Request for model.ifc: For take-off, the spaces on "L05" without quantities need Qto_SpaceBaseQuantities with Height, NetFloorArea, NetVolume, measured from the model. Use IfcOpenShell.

First a look at what the model holds.

```python
import ifcopenshell
import ifcopenshell.util.element
import ifcopenshell.util.unit

model = ifcopenshell.open("model.ifc")
print(model.schema)
for unit_type in ("LENGTHUNIT", "AREAUNIT", "VOLUMEUNIT"):
    print(unit_type, ifcopenshell.util.unit.calculate_unit_scale(model, unit_type))
storey = next(s for s in model.by_type("IfcBuildingStorey") if s.Name == "L05")
spaces = [e for e in ifcopenshell.util.element.get_decomposition(storey) if e.is_a("IfcSpace")]
for e in sorted(spaces, key=lambda e: e.id()):
    print(e.id(), e.is_a(), e.Name, list(ifcopenshell.util.element.get_psets(e, qtos_only=True)), sep=" | ")
```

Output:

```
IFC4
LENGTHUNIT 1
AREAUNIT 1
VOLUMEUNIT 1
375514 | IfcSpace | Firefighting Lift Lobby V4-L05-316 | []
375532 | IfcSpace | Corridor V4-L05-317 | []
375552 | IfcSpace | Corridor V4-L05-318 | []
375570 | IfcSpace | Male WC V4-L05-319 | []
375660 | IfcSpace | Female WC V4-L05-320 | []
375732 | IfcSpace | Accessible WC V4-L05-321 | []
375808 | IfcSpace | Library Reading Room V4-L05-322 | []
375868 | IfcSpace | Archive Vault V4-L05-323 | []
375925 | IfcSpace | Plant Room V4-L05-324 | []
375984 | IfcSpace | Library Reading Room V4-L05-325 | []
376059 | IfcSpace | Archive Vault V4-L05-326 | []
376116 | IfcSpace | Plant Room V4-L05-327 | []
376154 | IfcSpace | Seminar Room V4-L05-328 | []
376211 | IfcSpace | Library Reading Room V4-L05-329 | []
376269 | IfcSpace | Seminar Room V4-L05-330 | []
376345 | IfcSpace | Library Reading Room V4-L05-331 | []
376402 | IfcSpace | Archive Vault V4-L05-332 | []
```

```python
import ifcopenshell
import ifcopenshell.api.pset
import ifcopenshell.geom
import ifcopenshell.util.element
import ifcopenshell.util.shape
import ifcopenshell.util.unit

model = ifcopenshell.open("model.ifc")
unit_scale = ifcopenshell.util.unit.calculate_unit_scale(model)
area_scale = ifcopenshell.util.unit.calculate_unit_scale(model, "AREAUNIT")
volume_scale = ifcopenshell.util.unit.calculate_unit_scale(model, "VOLUMEUNIT")
settings = ifcopenshell.geom.settings()

storey = next(s for s in model.by_type("IfcBuildingStorey") if s.Name == "L05")
spaces = [e for e in ifcopenshell.util.element.get_decomposition(storey) if e.is_a("IfcSpace")]

for e in sorted(spaces, key=lambda e: e.id()):
    if ifcopenshell.util.element.get_psets(e, qtos_only=True, should_inherit=False):
        continue
    # Geometry comes back in metres, in the element's own axes.
    shape = ifcopenshell.geom.create_shape(settings, e)
    values = {
        "Height": ifcopenshell.util.shape.get_z(shape.geometry) / unit_scale,
        "NetFloorArea": ifcopenshell.util.shape.get_footprint_area(shape.geometry) / area_scale,
        "NetVolume": ifcopenshell.util.shape.get_volume(shape.geometry) / volume_scale,
    }
    qto = ifcopenshell.api.pset.add_qto(model, product=e, name="Qto_SpaceBaseQuantities")
    ifcopenshell.api.pset.edit_qto(model, qto=qto, properties=values)
    print(e.id(), {k: round(v, 3) for k, v in values.items()})

model.write("model_updated.ifc")
```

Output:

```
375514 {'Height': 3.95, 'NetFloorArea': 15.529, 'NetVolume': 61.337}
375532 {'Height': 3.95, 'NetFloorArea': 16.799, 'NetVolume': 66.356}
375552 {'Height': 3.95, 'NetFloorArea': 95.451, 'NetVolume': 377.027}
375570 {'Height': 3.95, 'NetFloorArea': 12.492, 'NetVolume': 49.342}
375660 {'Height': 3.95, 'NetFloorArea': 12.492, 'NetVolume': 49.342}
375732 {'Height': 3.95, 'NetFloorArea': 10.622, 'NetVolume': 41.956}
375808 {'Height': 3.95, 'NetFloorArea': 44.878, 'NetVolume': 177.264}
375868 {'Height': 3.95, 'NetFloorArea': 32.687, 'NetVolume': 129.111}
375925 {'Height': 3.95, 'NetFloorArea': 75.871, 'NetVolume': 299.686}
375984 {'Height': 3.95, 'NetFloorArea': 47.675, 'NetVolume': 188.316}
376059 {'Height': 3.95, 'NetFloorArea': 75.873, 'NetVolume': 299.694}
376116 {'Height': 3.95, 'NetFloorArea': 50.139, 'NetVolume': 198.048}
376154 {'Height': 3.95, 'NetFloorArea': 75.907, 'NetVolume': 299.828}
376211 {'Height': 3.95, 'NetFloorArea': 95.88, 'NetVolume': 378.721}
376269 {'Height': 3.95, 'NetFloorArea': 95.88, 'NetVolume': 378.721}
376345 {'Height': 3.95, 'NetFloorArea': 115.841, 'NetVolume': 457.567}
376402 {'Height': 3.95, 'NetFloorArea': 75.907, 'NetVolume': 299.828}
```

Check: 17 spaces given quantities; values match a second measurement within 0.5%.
